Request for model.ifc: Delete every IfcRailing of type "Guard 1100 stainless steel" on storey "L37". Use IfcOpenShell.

First a look at what the model holds.

```python
import ifcopenshell
import ifcopenshell.util.element

model = ifcopenshell.open("model.ifc")
print(model.schema)
storey = next(s for s in model.by_type("IfcBuildingStorey") if s.Name == "L37")
railings = [e for e in ifcopenshell.util.element.get_decomposition(storey) if e.is_a("IfcRailing")]
seen = {}
for e in railings:
    element_type = ifcopenshell.util.element.get_type(e)
    name = element_type.Name if element_type not in (None, e) else None
    seen[name] = seen.get(name, 0) + 1
for name, count in sorted(seen.items(), key=str):
    print(count, "x", name)
```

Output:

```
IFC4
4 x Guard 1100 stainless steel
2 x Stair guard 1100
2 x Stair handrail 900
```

```python
import ifcopenshell
import ifcopenshell.api.root
import ifcopenshell.util.element

model = ifcopenshell.open("model.ifc")

storey = next(s for s in model.by_type("IfcBuildingStorey") if s.Name == "L37")
railings = [e for e in ifcopenshell.util.element.get_decomposition(storey) if e.is_a("IfcRailing")]
targets = [e for e in railings if (t := ifcopenshell.util.element.get_type(e)) not in (None, e) and t.Name == "Guard 1100 stainless steel"]

for e in targets:
    ifcopenshell.api.root.remove_product(model, product=e)
print(len(targets), "removed")

model.write("model_rev.ifc")
```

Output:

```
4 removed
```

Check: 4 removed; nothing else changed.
